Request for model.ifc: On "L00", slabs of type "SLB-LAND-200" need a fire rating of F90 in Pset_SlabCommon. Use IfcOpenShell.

First a look at what the model holds.

```python
import ifcopenshell
import ifcopenshell.util.element

model = ifcopenshell.open("model.ifc")
print(model.schema)
storey = next(s for s in model.by_type("IfcBuildingStorey") if s.Name == "L00")
slabs = [e for e in ifcopenshell.util.element.get_decomposition(storey) if e.is_a("IfcSlab")]
seen = {}
for e in slabs:
    element_type = ifcopenshell.util.element.get_type(e)
    key = (element_type.Name if element_type != e and element_type else None, ifcopenshell.util.element.get_pset(e, "Pset_SlabCommon", "FireRating"))
    seen[key] = seen.get(key, 0) + 1
for (name, value), count in sorted(seen.items(), key=str):
    print(count, "x", name, "|", value)
```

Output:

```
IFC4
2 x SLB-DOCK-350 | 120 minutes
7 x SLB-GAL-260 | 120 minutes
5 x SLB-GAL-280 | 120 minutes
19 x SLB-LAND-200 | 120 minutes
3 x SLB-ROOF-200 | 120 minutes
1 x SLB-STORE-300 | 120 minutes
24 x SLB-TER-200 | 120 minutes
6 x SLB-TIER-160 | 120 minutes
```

```python
import ifcopenshell
import ifcopenshell.api.pset
import ifcopenshell.util.element

model = ifcopenshell.open("model.ifc")

storey = next(s for s in model.by_type("IfcBuildingStorey") if s.Name == "L00")
slabs = [e for e in ifcopenshell.util.element.get_decomposition(storey) if e.is_a("IfcSlab")]

count = 0
for e in slabs:
    element_type = ifcopenshell.util.element.get_type(e)
    if element_type in (None, e) or element_type.Name != "SLB-LAND-200":
        continue
    # add_pset returns the element's existing set when there is one.
    pset = ifcopenshell.api.pset.add_pset(model, product=e, name="Pset_SlabCommon")
    ifcopenshell.api.pset.edit_pset(model, pset=pset, properties={"FireRating": "F90"})
    count += 1

print(count, "slabs updated")

model.write("model_edited.ifc")
```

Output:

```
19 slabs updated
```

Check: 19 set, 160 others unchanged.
